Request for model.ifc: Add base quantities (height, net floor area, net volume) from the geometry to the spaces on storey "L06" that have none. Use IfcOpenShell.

First a look at what the model holds.

```python
import ifcopenshell
import ifcopenshell.util.element
import ifcopenshell.util.unit

model = ifcopenshell.open("model.ifc")
print(model.schema)
for unit_type in ("LENGTHUNIT", "AREAUNIT", "VOLUMEUNIT"):
    print(unit_type, ifcopenshell.util.unit.calculate_unit_scale(model, unit_type))
storey = next(s for s in model.by_type("IfcBuildingStorey") if s.Name == "L06")
spaces = [e for e in ifcopenshell.util.element.get_decomposition(storey) if e.is_a("IfcSpace")]
for e in sorted(spaces, key=lambda e: e.id()):
    print(e.id(), e.is_a(), e.Name, list(ifcopenshell.util.element.get_psets(e, qtos_only=True)), sep=" | ")
```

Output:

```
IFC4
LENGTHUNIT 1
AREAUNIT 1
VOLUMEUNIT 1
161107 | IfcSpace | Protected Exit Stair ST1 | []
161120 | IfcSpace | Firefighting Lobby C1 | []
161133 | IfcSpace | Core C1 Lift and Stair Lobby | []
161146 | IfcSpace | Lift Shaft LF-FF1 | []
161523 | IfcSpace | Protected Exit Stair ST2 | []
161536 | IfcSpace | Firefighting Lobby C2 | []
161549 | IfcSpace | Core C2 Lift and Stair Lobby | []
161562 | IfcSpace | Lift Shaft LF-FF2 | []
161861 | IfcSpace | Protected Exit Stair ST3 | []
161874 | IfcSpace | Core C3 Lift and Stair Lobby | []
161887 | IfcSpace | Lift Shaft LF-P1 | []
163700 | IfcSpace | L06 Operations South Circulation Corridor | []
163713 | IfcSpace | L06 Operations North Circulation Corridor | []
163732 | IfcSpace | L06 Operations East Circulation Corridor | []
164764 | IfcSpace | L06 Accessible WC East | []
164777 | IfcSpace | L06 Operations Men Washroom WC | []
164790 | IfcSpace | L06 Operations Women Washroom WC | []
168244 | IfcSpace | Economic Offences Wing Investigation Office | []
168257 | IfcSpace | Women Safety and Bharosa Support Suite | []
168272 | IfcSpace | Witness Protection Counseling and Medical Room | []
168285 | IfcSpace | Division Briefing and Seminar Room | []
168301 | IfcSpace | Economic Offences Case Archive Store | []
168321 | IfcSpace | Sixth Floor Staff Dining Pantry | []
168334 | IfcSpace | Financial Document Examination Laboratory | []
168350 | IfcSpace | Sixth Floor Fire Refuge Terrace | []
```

```python
import ifcopenshell
import ifcopenshell.api.pset
import ifcopenshell.geom
import ifcopenshell.util.element
import ifcopenshell.util.shape
import ifcopenshell.util.unit

model = ifcopenshell.open("model.ifc")
unit_scale = ifcopenshell.util.unit.calculate_unit_scale(model)
area_scale = ifcopenshell.util.unit.calculate_unit_scale(model, "AREAUNIT")
volume_scale = ifcopenshell.util.unit.calculate_unit_scale(model, "VOLUMEUNIT")
settings = ifcopenshell.geom.settings()

storey = next(s for s in model.by_type("IfcBuildingStorey") if s.Name == "L06")
spaces = [e for e in ifcopenshell.util.element.get_decomposition(storey) if e.is_a("IfcSpace")]

for e in sorted(spaces, key=lambda e: e.id()):
    if ifcopenshell.util.element.get_psets(e, qtos_only=True, should_inherit=False):
        continue
    # Geometry comes back in metres, in the element's own axes.
    shape = ifcopenshell.geom.create_shape(settings, e)
    values = {
        "Height": ifcopenshell.util.shape.get_z(shape.geometry) / unit_scale,
        "NetFloorArea": ifcopenshell.util.shape.get_footprint_area(shape.geometry) / area_scale,
        "NetVolume": ifcopenshell.util.shape.get_volume(shape.geometry) / volume_scale,
    }
    qto = ifcopenshell.api.pset.add_qto(model, product=e, name="Qto_SpaceBaseQuantities")
    ifcopenshell.api.pset.edit_qto(model, qto=qto, properties=values)
    print(e.id(), {k: round(v, 3) for k, v in values.items()})

model.write("model_rev.ifc")
```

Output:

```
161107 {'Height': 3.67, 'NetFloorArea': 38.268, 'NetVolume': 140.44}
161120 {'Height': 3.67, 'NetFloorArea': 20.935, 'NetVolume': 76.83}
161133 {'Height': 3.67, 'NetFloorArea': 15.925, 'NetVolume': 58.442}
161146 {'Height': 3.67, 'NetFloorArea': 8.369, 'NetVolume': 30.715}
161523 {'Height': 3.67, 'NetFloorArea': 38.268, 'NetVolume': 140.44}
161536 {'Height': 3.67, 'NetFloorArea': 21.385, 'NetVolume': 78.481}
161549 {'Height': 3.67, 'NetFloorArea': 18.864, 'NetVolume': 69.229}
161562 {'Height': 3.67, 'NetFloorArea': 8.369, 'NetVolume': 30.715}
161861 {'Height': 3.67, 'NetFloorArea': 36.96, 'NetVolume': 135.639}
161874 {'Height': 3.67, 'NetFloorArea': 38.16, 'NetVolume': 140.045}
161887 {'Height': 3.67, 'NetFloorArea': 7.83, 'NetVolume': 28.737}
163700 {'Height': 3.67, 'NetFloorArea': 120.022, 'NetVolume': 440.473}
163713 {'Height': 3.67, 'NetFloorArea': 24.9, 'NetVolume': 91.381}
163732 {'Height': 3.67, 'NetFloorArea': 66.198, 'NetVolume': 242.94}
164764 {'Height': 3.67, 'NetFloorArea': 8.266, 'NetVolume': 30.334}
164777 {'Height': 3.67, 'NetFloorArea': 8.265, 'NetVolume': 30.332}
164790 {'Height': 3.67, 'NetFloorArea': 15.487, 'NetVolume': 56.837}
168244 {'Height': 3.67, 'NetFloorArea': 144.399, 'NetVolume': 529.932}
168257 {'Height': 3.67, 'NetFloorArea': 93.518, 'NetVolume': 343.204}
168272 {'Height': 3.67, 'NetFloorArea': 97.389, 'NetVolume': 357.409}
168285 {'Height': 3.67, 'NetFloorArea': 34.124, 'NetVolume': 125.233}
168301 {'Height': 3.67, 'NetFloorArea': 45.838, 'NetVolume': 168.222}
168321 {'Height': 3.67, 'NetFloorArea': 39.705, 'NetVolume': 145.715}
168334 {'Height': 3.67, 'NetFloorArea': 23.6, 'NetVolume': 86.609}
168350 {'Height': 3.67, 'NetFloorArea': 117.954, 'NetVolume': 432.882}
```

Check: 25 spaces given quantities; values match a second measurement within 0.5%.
